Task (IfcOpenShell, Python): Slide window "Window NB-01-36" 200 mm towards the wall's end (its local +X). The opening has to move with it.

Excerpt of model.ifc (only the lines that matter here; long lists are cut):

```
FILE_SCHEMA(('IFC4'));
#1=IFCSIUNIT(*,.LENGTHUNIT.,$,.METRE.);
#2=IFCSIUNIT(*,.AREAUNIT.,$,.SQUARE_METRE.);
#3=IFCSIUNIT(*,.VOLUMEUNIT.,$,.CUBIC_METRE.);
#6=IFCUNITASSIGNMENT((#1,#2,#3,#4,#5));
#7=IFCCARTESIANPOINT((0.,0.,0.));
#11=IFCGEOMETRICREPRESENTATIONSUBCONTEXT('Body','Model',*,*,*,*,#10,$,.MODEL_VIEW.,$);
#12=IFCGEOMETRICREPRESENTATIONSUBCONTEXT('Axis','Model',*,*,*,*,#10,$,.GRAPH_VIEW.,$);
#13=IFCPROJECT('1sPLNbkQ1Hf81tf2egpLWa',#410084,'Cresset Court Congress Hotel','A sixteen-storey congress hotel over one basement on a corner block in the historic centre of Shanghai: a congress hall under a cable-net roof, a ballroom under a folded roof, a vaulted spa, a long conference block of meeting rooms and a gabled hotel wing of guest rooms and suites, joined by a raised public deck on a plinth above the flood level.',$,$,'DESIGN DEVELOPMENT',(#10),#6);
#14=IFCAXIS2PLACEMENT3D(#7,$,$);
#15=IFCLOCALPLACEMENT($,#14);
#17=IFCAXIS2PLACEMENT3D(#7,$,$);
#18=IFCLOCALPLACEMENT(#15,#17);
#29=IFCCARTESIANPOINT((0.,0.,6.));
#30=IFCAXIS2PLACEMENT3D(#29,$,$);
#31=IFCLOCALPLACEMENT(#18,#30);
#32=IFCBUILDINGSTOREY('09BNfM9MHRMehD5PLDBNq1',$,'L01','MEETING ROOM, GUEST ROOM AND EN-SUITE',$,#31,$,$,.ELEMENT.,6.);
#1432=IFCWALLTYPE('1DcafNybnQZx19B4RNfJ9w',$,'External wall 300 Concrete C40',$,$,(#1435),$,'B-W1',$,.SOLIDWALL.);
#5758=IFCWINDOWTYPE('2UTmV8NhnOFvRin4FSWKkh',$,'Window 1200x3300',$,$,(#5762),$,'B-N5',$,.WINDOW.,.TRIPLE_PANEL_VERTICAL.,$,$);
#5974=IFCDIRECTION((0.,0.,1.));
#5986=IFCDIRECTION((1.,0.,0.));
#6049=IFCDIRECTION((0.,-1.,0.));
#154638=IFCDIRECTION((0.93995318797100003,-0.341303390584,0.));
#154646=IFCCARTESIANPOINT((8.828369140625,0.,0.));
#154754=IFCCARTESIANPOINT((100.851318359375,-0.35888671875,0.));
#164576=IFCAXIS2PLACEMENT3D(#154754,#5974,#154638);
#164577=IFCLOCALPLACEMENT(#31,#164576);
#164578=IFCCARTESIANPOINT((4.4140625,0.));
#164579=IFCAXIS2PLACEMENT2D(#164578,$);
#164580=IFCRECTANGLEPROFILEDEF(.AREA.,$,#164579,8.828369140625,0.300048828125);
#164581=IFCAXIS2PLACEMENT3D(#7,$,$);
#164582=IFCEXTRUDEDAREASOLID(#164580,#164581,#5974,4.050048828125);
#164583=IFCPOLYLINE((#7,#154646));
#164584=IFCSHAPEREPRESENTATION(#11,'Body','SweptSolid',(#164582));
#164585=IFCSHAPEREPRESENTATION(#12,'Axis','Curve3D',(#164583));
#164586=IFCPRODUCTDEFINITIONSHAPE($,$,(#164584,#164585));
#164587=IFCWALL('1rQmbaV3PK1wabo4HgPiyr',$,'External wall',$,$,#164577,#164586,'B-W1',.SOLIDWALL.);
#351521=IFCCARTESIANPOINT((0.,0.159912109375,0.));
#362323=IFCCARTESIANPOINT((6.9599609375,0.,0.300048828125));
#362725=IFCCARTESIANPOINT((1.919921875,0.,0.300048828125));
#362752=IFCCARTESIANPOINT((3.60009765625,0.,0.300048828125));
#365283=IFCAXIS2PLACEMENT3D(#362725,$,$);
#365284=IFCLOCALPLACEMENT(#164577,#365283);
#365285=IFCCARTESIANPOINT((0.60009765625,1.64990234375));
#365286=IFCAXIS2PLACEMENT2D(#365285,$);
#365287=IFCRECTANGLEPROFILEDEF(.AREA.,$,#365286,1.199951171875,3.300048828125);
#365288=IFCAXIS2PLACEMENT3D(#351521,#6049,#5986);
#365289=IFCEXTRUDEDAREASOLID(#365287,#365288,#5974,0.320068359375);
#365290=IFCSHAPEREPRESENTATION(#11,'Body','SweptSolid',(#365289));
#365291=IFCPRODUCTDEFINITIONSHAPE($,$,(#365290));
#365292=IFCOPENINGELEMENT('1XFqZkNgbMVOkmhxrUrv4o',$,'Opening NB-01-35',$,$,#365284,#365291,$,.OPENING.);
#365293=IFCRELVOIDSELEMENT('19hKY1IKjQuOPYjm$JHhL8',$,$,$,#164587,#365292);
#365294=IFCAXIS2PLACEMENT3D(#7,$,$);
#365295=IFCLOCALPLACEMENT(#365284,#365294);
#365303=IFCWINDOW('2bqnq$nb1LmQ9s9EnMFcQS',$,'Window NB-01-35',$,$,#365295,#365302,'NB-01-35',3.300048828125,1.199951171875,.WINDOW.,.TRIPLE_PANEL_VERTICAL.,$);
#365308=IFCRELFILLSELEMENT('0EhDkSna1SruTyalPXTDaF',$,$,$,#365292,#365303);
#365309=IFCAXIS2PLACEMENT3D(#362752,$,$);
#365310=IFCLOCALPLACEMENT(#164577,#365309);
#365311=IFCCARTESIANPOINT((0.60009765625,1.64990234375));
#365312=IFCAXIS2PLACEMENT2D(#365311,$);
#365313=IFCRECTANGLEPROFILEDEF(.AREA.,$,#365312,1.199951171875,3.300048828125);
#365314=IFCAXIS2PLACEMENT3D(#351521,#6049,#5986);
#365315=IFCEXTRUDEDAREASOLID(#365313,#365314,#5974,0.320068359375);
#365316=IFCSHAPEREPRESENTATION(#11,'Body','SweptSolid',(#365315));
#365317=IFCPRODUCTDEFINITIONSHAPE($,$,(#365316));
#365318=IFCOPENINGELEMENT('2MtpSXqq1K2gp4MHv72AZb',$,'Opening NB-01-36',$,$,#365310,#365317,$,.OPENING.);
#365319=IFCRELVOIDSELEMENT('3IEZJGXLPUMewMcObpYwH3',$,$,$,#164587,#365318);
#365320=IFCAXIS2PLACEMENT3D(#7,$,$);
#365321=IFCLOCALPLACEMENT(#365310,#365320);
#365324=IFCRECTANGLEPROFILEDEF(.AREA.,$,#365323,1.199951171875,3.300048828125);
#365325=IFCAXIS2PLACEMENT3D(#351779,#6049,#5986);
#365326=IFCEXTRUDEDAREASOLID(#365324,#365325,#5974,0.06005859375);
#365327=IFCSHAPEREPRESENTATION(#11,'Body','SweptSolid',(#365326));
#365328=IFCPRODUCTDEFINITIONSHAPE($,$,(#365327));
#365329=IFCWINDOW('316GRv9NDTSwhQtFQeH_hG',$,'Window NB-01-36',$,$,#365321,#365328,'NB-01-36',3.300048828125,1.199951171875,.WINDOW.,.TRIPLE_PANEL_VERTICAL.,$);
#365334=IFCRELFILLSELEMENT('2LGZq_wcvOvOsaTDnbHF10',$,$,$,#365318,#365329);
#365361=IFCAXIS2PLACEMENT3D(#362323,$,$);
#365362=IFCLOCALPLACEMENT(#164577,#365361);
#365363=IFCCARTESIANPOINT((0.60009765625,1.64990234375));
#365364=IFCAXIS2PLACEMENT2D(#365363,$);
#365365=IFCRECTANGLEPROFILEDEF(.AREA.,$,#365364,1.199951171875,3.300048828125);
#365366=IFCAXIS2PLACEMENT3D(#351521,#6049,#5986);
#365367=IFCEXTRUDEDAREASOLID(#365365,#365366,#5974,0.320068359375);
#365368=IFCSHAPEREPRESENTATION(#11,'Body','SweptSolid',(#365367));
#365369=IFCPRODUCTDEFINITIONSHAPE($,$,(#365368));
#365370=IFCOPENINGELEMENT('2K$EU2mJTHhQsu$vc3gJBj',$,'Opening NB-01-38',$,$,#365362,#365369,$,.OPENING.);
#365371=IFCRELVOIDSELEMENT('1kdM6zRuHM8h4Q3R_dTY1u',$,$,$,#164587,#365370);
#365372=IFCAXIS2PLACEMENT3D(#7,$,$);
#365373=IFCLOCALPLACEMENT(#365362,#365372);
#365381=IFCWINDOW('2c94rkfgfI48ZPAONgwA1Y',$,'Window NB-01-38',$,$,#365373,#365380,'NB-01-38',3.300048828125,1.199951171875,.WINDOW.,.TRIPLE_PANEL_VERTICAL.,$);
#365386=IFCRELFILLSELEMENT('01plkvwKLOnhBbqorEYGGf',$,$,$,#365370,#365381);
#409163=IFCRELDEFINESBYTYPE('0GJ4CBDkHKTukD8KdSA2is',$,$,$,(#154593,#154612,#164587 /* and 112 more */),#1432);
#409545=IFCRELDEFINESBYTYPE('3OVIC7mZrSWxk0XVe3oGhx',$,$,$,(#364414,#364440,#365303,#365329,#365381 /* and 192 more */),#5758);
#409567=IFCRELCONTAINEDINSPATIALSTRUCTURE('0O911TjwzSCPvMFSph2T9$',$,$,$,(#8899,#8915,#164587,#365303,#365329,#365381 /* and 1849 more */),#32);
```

```python
import ifcopenshell
import ifcopenshell.api.geometry
import ifcopenshell.util.placement
import ifcopenshell.util.unit

model = ifcopenshell.open("model.ifc")
unit_scale = ifcopenshell.util.unit.calculate_unit_scale(model)

window = model.by_guid("316GRv9NDTSwhQtFQeH_hG")
opening = window.FillsVoids[0].RelatingOpeningElement
wall = opening.VoidsElements[0].RelatingBuildingElement

wall_matrix = ifcopenshell.util.placement.get_local_placement(wall.ObjectPlacement)
shift = wall_matrix[:3, 0] * 0.2 / unit_scale
before = ifcopenshell.util.placement.get_local_placement(window.ObjectPlacement)[:3, 3].copy()

# The window is placed relative to its opening, so it follows when the opening moves.
matrix = ifcopenshell.util.placement.get_local_placement(opening.ObjectPlacement)
matrix[:3, 3] += shift
ifcopenshell.api.geometry.edit_object_placement(
    model, product=opening, matrix=matrix, is_si=False, should_transform_children=True
)

after = ifcopenshell.util.placement.get_local_placement(window.ObjectPlacement)[:3, 3]
print("window moved by", (after - before).round(3) + 0.0)

model.write("model_rev.ifc")
```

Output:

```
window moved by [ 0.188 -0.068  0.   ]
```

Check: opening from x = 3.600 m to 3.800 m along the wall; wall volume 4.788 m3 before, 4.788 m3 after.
